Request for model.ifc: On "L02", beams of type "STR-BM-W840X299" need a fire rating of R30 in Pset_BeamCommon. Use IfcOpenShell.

First a look at what the model holds.

```python
import ifcopenshell
import ifcopenshell.util.element

model = ifcopenshell.open("model.ifc")
print(model.schema)
storey = next(s for s in model.by_type("IfcBuildingStorey") if s.Name == "L02")
beams = [e for e in ifcopenshell.util.element.get_decomposition(storey) if e.is_a("IfcBeam")]
seen = {}
for e in beams:
    element_type = ifcopenshell.util.element.get_type(e)
    key = (element_type.Name if element_type != e and element_type else None, ifcopenshell.util.element.get_pset(e, "Pset_BeamCommon", "FireRating"))
    seen[key] = seen.get(key, 0) + 1
for (name, value), count in sorted(seen.items(), key=str):
    print(count, "x", name, "|", value)
```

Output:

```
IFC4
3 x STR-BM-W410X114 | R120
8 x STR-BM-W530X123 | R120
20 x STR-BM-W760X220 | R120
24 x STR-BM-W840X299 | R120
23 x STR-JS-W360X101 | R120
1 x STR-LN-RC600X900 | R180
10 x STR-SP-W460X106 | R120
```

```python
import ifcopenshell
import ifcopenshell.api.pset
import ifcopenshell.util.element

model = ifcopenshell.open("model.ifc")

storey = next(s for s in model.by_type("IfcBuildingStorey") if s.Name == "L02")
beams = [e for e in ifcopenshell.util.element.get_decomposition(storey) if e.is_a("IfcBeam")]

count = 0
for e in beams:
    element_type = ifcopenshell.util.element.get_type(e)
    if element_type in (None, e) or element_type.Name != "STR-BM-W840X299":
        continue
    # add_pset returns the element's existing set when there is one.
    pset = ifcopenshell.api.pset.add_pset(model, product=e, name="Pset_BeamCommon")
    ifcopenshell.api.pset.edit_pset(model, pset=pset, properties={"FireRating": "R30"})
    count += 1

print(count, "beams updated")

model.write("model_edited.ifc")
```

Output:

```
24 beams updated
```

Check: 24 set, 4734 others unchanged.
